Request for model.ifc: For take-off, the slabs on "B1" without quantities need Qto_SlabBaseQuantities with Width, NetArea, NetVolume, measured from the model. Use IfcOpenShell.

First a look at what the model holds.

```python
import ifcopenshell
import ifcopenshell.util.element
import ifcopenshell.util.unit

model = ifcopenshell.open("model.ifc")
print(model.schema)
for unit_type in ("LENGTHUNIT", "AREAUNIT", "VOLUMEUNIT"):
    print(unit_type, ifcopenshell.util.unit.calculate_unit_scale(model, unit_type))
storey = next(s for s in model.by_type("IfcBuildingStorey") if s.Name == "B1")
slabs = [e for e in ifcopenshell.util.element.get_decomposition(storey) if e.is_a("IfcSlab")]
for e in sorted(slabs, key=lambda e: e.id()):
    print(e.id(), e.is_a(), e.Name, list(ifcopenshell.util.element.get_psets(e, qtos_only=True)), sep=" | ")
```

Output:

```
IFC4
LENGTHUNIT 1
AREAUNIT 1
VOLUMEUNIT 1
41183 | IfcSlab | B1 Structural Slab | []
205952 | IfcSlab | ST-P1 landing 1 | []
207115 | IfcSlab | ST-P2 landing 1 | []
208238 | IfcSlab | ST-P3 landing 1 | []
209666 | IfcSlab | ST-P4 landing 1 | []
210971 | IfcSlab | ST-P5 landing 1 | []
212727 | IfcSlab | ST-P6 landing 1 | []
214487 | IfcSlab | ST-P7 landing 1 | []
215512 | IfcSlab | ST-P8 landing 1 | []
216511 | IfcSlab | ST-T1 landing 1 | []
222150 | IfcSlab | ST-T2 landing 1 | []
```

```python
import ifcopenshell
import ifcopenshell.api.pset
import ifcopenshell.geom
import ifcopenshell.util.element
import ifcopenshell.util.shape
import ifcopenshell.util.unit

model = ifcopenshell.open("model.ifc")
unit_scale = ifcopenshell.util.unit.calculate_unit_scale(model)
area_scale = ifcopenshell.util.unit.calculate_unit_scale(model, "AREAUNIT")
volume_scale = ifcopenshell.util.unit.calculate_unit_scale(model, "VOLUMEUNIT")
settings = ifcopenshell.geom.settings()

storey = next(s for s in model.by_type("IfcBuildingStorey") if s.Name == "B1")
slabs = [e for e in ifcopenshell.util.element.get_decomposition(storey) if e.is_a("IfcSlab")]

for e in sorted(slabs, key=lambda e: e.id()):
    if ifcopenshell.util.element.get_psets(e, qtos_only=True, should_inherit=False):
        continue
    # Geometry comes back in metres, in the element's own axes.
    shape = ifcopenshell.geom.create_shape(settings, e)
    values = {
        "Width": ifcopenshell.util.shape.get_z(shape.geometry) / unit_scale,
        "NetArea": ifcopenshell.util.shape.get_footprint_area(shape.geometry) / area_scale,
        "NetVolume": ifcopenshell.util.shape.get_volume(shape.geometry) / volume_scale,
    }
    qto = ifcopenshell.api.pset.add_qto(model, product=e, name="Qto_SlabBaseQuantities")
    ifcopenshell.api.pset.edit_qto(model, qto=qto, properties=values)
    print(e.id(), {k: round(v, 3) for k, v in values.items()})

model.write("model_v2.ifc")
```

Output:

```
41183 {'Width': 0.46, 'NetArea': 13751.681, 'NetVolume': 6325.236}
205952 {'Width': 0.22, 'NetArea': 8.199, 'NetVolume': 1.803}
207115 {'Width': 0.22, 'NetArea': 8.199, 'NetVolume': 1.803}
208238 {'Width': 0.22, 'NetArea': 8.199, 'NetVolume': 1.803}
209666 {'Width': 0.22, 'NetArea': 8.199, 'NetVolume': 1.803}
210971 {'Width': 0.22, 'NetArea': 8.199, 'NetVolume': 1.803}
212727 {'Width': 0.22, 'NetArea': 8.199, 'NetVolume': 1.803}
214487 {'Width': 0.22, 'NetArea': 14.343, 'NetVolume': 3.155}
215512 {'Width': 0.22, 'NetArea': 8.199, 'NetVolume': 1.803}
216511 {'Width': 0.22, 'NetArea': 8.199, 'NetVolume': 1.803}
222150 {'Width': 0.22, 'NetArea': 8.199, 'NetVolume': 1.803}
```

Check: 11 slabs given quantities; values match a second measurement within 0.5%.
